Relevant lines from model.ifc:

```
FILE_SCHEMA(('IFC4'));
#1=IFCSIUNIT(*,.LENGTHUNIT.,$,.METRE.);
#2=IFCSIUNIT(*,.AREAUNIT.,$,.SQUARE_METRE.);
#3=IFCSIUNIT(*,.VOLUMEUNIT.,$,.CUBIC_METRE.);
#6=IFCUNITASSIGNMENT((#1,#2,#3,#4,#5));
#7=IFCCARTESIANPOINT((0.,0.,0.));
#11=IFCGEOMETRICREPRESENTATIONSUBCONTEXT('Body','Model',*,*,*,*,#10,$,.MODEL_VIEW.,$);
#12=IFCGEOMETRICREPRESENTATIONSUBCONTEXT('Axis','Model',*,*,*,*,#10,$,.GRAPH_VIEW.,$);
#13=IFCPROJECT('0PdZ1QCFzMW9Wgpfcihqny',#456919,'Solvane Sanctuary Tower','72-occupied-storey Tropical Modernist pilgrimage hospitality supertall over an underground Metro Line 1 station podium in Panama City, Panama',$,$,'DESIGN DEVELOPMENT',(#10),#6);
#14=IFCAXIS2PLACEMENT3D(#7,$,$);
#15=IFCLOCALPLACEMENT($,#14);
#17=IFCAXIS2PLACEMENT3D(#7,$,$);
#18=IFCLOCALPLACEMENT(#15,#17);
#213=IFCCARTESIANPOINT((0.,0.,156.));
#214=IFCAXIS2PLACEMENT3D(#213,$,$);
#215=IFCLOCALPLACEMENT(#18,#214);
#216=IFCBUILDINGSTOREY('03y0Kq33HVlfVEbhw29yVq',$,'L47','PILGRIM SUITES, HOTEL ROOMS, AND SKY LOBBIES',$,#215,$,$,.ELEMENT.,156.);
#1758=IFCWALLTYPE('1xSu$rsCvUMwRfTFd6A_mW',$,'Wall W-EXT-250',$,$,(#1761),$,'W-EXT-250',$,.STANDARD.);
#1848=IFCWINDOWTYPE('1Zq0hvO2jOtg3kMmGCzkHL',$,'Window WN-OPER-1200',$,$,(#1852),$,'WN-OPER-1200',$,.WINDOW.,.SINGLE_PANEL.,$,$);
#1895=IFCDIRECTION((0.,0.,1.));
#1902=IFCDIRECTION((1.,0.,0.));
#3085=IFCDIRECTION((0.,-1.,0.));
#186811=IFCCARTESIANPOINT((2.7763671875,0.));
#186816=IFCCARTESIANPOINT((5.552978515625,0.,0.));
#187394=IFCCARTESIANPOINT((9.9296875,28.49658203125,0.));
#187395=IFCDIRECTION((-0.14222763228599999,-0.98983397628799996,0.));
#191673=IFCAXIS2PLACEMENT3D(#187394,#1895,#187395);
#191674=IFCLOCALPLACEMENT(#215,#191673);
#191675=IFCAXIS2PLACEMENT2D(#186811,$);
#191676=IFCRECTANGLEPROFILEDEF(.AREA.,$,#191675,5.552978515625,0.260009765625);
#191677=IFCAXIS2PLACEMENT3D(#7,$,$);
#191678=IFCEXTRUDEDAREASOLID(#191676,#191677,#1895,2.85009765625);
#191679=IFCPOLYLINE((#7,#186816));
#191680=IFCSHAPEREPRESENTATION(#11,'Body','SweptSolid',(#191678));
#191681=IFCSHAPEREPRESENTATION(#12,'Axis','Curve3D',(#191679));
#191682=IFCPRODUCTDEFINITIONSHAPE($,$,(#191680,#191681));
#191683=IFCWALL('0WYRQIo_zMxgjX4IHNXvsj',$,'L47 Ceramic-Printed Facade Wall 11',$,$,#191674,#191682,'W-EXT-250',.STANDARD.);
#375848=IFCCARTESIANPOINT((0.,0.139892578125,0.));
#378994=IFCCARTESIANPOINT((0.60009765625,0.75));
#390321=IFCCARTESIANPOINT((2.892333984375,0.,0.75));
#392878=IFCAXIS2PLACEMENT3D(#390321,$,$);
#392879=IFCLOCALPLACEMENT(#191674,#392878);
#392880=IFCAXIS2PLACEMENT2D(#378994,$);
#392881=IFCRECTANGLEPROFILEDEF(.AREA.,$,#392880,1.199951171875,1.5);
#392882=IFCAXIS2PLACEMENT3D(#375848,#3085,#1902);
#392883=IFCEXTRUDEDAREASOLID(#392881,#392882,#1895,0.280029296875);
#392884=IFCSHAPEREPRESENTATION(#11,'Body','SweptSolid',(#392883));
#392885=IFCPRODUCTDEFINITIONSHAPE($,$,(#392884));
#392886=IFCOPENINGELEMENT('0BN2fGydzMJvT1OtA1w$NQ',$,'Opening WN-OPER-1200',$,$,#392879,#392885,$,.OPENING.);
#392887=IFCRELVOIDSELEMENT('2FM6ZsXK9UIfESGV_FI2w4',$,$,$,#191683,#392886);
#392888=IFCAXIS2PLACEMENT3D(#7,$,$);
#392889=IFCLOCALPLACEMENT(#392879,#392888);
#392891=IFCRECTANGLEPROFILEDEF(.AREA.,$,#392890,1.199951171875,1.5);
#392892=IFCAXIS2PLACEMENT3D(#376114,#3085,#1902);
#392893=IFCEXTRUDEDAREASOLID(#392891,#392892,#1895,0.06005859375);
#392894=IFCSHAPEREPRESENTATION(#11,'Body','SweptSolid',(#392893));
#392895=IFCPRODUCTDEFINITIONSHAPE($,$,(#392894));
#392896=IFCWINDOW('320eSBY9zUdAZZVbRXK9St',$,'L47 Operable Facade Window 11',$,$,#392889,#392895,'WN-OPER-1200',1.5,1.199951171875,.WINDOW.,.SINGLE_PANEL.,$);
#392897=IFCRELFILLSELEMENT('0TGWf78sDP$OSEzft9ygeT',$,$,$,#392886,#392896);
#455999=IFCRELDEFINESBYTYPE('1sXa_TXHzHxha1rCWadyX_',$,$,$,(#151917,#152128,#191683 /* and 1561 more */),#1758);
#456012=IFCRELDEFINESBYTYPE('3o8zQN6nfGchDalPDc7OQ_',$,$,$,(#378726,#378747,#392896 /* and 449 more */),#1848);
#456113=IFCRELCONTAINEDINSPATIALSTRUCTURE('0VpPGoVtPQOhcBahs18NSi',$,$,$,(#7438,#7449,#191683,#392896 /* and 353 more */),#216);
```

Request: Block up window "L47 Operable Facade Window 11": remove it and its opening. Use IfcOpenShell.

```python
import ifcopenshell
import ifcopenshell.api.feature
import ifcopenshell.api.root
import ifcopenshell.geom
import ifcopenshell.util.shape

model = ifcopenshell.open("model.ifc")
settings = ifcopenshell.geom.settings()


def volume(element):
    """Net volume in cubic metres, openings subtracted."""
    shape = ifcopenshell.geom.create_shape(settings, element)
    return ifcopenshell.util.shape.get_volume(shape.geometry)


window = model.by_guid("320eSBY9zUdAZZVbRXK9St")
opening = window.FillsVoids[0].RelatingOpeningElement
wall = opening.VoidsElements[0].RelatingBuildingElement
before = volume(wall)

ifcopenshell.api.root.remove_product(model, product=window)
ifcopenshell.api.feature.remove_feature(model, feature=opening)

after = volume(wall)

print(f"wall volume {before:.3f} -> {after:.3f} m3")

model.write("model_v2.ifc")
```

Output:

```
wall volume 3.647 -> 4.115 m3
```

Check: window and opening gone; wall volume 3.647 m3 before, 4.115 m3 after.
